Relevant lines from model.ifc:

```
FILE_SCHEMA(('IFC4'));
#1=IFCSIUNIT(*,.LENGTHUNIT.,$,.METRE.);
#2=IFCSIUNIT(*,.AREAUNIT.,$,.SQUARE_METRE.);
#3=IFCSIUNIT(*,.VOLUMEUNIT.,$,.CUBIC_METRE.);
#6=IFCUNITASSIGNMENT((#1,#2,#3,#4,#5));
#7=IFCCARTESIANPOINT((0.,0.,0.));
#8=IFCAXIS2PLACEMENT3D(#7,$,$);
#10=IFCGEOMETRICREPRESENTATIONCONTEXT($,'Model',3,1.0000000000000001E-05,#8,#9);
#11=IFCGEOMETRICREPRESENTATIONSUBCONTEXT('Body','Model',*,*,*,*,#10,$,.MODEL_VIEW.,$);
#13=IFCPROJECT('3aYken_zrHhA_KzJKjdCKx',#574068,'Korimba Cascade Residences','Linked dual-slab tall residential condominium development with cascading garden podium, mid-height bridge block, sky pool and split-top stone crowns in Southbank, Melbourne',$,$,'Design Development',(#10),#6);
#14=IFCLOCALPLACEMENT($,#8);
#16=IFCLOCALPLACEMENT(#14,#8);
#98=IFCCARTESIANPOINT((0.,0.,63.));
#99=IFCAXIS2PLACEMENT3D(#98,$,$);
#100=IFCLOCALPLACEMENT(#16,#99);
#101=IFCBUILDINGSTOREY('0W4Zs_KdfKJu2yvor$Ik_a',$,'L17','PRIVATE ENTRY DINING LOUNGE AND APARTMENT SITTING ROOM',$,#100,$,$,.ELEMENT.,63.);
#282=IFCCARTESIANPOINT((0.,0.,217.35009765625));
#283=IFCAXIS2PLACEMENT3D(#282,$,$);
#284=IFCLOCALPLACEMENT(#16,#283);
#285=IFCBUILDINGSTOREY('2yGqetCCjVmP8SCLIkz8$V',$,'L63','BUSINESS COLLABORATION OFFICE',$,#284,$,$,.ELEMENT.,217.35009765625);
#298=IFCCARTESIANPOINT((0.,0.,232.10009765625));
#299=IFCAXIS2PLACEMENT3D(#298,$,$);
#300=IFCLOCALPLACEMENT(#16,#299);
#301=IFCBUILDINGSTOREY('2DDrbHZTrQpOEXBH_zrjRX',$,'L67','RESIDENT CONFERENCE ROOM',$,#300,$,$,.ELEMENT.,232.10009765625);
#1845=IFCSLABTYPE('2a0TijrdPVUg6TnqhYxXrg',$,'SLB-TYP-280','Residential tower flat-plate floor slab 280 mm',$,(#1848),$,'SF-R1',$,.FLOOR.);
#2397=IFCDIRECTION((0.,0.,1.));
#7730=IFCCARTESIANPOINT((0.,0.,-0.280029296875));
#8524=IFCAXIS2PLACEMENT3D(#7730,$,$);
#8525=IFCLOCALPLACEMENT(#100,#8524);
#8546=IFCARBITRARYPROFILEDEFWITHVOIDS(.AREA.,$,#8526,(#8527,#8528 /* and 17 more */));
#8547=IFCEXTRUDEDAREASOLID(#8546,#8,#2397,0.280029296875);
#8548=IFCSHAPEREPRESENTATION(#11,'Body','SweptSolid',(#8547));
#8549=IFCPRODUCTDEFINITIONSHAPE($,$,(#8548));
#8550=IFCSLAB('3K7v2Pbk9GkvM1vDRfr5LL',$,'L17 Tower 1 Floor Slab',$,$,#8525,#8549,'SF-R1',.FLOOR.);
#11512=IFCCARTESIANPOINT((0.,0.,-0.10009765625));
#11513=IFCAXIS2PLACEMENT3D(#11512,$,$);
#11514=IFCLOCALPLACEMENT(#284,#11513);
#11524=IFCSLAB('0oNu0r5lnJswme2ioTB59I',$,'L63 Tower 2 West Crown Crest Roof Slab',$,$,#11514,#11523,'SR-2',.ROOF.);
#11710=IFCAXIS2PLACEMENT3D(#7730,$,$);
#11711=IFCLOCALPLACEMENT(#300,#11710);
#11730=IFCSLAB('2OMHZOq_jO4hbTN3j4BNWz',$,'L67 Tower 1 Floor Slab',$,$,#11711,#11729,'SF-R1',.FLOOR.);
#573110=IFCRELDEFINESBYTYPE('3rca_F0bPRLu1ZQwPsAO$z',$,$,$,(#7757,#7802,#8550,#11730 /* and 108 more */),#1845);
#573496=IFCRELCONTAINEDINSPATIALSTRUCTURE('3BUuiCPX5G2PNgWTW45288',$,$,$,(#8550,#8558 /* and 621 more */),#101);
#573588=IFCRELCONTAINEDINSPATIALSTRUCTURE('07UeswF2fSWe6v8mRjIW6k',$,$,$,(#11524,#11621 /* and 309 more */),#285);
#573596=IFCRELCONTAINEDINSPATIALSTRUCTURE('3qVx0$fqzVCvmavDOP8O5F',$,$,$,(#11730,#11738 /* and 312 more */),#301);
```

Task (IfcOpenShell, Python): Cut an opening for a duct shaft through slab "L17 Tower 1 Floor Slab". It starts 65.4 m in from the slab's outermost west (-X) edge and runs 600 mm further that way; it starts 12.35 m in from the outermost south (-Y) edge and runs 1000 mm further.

```python
import numpy as np
import ifcopenshell
import ifcopenshell.api.feature
import ifcopenshell.api.geometry
import ifcopenshell.api.root
import ifcopenshell.geom
import ifcopenshell.util.placement
import ifcopenshell.util.representation
import ifcopenshell.util.shape
import ifcopenshell.util.unit

model = ifcopenshell.open("model.ifc")
unit_scale = ifcopenshell.util.unit.calculate_unit_scale(model)
settings = ifcopenshell.geom.settings()


def volume(element):
    """Net volume in cubic metres, openings subtracted."""
    shape = ifcopenshell.geom.create_shape(settings, element)
    return ifcopenshell.util.shape.get_volume(shape.geometry)


slab = model.by_id(8550)
before = volume(slab)

# Extent in the slab's own axes, in metres. The edges named are its -X and -Y sides.
slab_shape = ifcopenshell.geom.create_shape(settings, slab)
vertices = ifcopenshell.util.shape.get_vertices(slab_shape.geometry)
x_min, y_min, bottom = vertices.min(axis=0)
top = vertices[:, 2].max()

opening = ifcopenshell.api.root.create_entity(model, ifc_class="IfcOpeningElement", name="Duct shaft opening", predefined_type="OPENING")
context = ifcopenshell.util.representation.get_context(model, "Model", "Body", "MODEL_VIEW")
width, depth = 0.6, 1
outline = [(0.0, 0.0), (width, 0.0), (width, depth), (0.0, depth), (0.0, 0.0)]
# Overshoot both faces by 50 mm so the cut is clean.
shape = ifcopenshell.api.geometry.add_slab_representation(
    model, context=context, depth=top - bottom + 0.1, polyline=outline
)
ifcopenshell.api.geometry.assign_representation(model, product=opening, representation=shape)

matrix = ifcopenshell.util.placement.get_local_placement(slab.ObjectPlacement)
matrix[:, 3] = matrix @ np.append(np.array([x_min + 65.4, y_min + 12.35, bottom - 0.05]) / unit_scale, 1.0)
ifcopenshell.api.geometry.edit_object_placement(model, product=opening, matrix=matrix, is_si=False)
ifcopenshell.api.feature.add_feature(model, feature=opening, element=slab)

after = volume(slab)

print(f"slab volume {before:.3f} -> {after:.3f} m3")

model.write("model_updated.ifc")
```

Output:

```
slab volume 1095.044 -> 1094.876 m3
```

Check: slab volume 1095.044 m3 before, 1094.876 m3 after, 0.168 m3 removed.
